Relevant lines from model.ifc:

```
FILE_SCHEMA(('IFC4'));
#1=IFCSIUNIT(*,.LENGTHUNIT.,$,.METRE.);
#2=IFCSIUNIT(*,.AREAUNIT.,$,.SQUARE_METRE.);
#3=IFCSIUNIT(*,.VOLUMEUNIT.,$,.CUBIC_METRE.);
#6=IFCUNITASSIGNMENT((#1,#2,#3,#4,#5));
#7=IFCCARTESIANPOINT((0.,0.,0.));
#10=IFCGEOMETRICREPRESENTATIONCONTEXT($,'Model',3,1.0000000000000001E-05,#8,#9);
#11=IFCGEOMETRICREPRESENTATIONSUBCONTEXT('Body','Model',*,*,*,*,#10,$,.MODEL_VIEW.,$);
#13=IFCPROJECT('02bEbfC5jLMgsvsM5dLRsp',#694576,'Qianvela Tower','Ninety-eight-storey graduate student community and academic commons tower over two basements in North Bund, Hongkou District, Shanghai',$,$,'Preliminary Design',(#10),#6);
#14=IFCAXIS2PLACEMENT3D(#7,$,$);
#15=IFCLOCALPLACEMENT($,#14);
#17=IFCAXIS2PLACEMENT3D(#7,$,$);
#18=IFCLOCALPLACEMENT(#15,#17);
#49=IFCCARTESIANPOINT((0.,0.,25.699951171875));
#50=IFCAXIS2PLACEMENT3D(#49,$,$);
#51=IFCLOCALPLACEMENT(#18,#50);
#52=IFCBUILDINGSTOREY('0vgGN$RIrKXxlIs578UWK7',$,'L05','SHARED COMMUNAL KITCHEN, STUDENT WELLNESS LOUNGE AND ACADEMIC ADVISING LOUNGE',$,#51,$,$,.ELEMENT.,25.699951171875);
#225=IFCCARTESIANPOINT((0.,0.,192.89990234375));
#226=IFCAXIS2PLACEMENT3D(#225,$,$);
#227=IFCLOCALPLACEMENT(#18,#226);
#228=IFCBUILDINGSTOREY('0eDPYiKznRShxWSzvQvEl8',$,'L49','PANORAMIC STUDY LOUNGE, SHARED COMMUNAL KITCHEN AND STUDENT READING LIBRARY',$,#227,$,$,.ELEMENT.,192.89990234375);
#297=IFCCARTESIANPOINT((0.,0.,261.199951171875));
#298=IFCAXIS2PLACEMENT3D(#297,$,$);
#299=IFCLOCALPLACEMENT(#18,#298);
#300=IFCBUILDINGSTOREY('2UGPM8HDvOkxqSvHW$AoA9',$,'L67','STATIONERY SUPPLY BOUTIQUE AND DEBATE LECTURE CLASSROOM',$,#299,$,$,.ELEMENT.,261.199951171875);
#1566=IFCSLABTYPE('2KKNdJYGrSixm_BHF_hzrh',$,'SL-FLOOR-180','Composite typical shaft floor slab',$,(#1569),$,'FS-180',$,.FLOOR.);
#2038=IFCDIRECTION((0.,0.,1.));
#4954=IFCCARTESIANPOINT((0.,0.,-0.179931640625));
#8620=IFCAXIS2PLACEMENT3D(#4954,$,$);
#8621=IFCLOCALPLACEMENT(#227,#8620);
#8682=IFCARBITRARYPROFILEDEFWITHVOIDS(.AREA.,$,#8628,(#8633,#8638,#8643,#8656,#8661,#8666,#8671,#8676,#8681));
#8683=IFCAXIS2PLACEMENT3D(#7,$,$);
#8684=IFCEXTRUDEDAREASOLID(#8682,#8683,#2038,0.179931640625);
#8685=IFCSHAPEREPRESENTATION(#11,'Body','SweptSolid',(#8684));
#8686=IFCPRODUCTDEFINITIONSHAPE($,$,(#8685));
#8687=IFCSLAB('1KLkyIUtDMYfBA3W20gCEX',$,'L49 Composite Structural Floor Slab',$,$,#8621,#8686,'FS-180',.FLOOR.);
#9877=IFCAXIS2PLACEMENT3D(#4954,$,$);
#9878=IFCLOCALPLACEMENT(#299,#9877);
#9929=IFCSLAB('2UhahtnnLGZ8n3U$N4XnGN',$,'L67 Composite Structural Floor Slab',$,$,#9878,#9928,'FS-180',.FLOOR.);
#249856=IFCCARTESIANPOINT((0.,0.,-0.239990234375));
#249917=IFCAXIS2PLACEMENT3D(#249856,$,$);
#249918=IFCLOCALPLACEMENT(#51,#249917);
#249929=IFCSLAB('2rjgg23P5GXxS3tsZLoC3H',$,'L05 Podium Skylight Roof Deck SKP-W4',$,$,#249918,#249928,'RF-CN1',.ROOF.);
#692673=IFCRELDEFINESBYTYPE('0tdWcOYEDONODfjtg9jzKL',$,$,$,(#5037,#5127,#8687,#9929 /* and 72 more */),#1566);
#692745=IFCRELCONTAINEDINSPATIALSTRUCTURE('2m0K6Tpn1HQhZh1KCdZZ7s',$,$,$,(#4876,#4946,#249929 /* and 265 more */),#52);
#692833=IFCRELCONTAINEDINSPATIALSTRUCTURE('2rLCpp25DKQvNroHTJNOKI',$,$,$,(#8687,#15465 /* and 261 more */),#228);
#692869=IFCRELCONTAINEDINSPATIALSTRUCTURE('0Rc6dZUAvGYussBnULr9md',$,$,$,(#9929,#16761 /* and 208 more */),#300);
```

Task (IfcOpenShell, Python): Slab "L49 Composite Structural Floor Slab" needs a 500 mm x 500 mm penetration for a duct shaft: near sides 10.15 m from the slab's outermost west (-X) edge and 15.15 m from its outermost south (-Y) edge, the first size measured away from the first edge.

```python
import numpy as np
import ifcopenshell
import ifcopenshell.api.feature
import ifcopenshell.api.geometry
import ifcopenshell.api.root
import ifcopenshell.geom
import ifcopenshell.util.placement
import ifcopenshell.util.representation
import ifcopenshell.util.shape
import ifcopenshell.util.unit

model = ifcopenshell.open("model.ifc")
unit_scale = ifcopenshell.util.unit.calculate_unit_scale(model)
settings = ifcopenshell.geom.settings()


def volume(element):
    """Net volume in cubic metres, openings subtracted."""
    shape = ifcopenshell.geom.create_shape(settings, element)
    return ifcopenshell.util.shape.get_volume(shape.geometry)


slab = model.by_guid("1KLkyIUtDMYfBA3W20gCEX")
before = volume(slab)

# Extent in the slab's own axes, in metres. The edges named are its -X and -Y sides.
slab_shape = ifcopenshell.geom.create_shape(settings, slab)
vertices = ifcopenshell.util.shape.get_vertices(slab_shape.geometry)
x_min, y_min, bottom = vertices.min(axis=0)
top = vertices[:, 2].max()

opening = ifcopenshell.api.root.create_entity(model, ifc_class="IfcOpeningElement", name="Duct shaft opening", predefined_type="OPENING")
context = ifcopenshell.util.representation.get_context(model, "Model", "Body", "MODEL_VIEW")
width, depth = 0.5, 0.5
outline = [(0.0, 0.0), (width, 0.0), (width, depth), (0.0, depth), (0.0, 0.0)]
# Overshoot both faces by 50 mm so the cut is clean.
shape = ifcopenshell.api.geometry.add_slab_representation(
    model, context=context, depth=top - bottom + 0.1, polyline=outline
)
ifcopenshell.api.geometry.assign_representation(model, product=opening, representation=shape)

matrix = ifcopenshell.util.placement.get_local_placement(slab.ObjectPlacement)
matrix[:, 3] = matrix @ np.append(np.array([x_min + 10.15, y_min + 15.15, bottom - 0.05]) / unit_scale, 1.0)
ifcopenshell.api.geometry.edit_object_placement(model, product=opening, matrix=matrix, is_si=False)
ifcopenshell.api.feature.add_feature(model, feature=opening, element=slab)

after = volume(slab)

print(f"slab volume {before:.3f} -> {after:.3f} m3")

model.write("model_rev.ifc")
```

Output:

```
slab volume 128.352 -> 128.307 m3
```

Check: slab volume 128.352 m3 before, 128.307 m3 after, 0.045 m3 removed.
